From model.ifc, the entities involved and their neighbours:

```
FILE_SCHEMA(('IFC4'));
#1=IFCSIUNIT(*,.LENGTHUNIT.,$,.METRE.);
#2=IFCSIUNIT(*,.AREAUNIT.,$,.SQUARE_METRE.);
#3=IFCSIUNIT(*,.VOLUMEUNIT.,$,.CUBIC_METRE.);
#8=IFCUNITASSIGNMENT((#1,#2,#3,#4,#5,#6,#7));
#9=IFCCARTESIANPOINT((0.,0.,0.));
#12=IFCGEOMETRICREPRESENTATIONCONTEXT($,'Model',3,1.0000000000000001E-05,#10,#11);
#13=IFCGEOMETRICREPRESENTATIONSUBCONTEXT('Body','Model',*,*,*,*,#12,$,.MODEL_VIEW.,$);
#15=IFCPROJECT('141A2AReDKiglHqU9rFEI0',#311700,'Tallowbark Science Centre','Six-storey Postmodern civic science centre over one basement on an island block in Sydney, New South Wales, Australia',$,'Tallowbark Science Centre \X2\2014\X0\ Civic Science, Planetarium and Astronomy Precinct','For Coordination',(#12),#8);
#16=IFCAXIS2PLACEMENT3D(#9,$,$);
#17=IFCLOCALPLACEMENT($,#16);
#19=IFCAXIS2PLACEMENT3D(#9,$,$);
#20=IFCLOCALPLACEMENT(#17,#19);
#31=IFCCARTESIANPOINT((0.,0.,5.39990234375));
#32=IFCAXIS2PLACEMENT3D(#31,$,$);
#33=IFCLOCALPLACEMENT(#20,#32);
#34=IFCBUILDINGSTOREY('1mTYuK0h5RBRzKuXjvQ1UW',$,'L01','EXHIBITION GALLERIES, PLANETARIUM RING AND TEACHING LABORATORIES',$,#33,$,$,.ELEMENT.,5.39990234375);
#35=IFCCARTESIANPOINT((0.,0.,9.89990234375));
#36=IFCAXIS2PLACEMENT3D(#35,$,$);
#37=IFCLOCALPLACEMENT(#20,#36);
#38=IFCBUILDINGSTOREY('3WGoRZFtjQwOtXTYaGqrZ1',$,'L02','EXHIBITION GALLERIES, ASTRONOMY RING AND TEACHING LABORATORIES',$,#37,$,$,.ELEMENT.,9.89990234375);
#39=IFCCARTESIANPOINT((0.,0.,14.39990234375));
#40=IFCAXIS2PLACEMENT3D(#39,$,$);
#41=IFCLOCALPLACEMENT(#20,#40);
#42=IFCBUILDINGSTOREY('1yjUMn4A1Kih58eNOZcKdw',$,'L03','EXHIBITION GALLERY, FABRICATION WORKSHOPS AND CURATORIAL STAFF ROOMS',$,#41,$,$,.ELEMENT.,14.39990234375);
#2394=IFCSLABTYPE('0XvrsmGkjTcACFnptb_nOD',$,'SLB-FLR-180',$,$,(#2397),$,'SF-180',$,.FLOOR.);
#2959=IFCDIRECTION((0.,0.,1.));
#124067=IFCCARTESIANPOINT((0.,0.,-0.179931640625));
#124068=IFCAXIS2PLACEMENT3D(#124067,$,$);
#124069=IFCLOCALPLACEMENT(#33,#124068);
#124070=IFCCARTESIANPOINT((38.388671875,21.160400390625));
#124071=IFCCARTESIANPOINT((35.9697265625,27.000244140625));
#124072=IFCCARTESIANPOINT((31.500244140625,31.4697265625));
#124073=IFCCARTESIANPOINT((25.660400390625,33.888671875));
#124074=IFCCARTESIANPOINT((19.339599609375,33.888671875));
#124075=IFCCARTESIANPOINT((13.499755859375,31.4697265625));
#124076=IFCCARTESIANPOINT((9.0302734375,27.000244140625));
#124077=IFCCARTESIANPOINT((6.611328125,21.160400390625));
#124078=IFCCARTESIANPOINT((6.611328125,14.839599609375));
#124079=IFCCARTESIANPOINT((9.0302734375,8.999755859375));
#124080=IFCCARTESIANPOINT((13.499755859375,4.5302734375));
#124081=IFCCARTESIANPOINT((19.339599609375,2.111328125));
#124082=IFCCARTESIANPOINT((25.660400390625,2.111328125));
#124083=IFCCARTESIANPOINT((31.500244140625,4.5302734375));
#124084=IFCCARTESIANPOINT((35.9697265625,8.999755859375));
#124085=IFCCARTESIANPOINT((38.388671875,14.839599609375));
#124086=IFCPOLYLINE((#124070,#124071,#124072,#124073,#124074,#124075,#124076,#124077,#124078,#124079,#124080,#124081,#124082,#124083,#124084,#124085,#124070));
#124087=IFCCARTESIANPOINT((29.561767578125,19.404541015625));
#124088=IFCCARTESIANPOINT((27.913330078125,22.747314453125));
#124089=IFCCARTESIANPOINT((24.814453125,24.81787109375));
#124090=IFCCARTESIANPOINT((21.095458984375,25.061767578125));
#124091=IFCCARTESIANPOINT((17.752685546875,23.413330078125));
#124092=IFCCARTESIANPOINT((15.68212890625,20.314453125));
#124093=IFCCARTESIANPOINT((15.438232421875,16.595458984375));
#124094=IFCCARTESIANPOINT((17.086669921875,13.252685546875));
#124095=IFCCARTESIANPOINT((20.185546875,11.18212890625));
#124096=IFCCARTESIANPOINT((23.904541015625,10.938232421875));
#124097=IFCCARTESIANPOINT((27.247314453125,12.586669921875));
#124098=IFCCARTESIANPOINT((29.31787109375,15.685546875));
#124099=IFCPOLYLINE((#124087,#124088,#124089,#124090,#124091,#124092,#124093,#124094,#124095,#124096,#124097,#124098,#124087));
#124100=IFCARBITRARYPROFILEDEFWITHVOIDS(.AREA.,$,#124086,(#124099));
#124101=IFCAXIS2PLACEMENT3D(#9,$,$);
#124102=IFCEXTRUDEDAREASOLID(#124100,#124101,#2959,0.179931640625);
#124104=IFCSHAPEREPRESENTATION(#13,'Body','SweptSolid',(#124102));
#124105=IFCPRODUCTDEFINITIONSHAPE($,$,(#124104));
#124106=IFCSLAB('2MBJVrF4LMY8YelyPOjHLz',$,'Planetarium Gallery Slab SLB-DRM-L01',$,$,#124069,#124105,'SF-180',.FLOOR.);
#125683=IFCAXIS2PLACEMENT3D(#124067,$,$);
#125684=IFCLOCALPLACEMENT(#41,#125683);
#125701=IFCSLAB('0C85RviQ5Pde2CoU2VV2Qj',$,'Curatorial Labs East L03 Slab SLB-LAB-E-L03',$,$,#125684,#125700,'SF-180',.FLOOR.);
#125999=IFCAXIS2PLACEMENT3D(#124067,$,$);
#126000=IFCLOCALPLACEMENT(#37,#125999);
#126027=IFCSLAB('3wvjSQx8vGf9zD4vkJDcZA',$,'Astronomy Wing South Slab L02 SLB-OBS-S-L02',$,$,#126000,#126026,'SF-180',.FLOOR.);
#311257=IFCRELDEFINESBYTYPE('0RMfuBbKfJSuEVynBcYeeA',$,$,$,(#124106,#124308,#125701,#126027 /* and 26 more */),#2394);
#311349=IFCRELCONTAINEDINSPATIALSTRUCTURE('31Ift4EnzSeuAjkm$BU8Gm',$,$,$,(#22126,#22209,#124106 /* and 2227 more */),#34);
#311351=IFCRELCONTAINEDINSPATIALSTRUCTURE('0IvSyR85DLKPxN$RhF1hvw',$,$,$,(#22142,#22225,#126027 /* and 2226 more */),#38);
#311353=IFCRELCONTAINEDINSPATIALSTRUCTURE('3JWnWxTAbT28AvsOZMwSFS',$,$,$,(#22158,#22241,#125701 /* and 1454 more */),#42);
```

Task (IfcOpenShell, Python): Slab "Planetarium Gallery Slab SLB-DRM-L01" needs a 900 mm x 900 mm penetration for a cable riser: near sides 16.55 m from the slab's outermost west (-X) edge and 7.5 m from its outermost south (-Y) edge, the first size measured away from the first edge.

```python
import numpy as np
import ifcopenshell
import ifcopenshell.api.feature
import ifcopenshell.api.geometry
import ifcopenshell.api.root
import ifcopenshell.geom
import ifcopenshell.util.placement
import ifcopenshell.util.representation
import ifcopenshell.util.shape
import ifcopenshell.util.unit

model = ifcopenshell.open("model.ifc")
unit_scale = ifcopenshell.util.unit.calculate_unit_scale(model)
settings = ifcopenshell.geom.settings()


def volume(element):
    """Net volume in cubic metres, openings subtracted."""
    shape = ifcopenshell.geom.create_shape(settings, element)
    return ifcopenshell.util.shape.get_volume(shape.geometry)


slab = model.by_guid("2MBJVrF4LMY8YelyPOjHLz")
before = volume(slab)

# Extent in the slab's own axes, in metres. The edges named are its -X and -Y sides.
slab_shape = ifcopenshell.geom.create_shape(settings, slab)
vertices = ifcopenshell.util.shape.get_vertices(slab_shape.geometry)
x_min, y_min, bottom = vertices.min(axis=0)
top = vertices[:, 2].max()

opening = ifcopenshell.api.root.create_entity(model, ifc_class="IfcOpeningElement", name="Cable riser opening", predefined_type="OPENING")
context = ifcopenshell.util.representation.get_context(model, "Model", "Body", "MODEL_VIEW")
width, depth = 0.9, 0.9
outline = [(0.0, 0.0), (width, 0.0), (width, depth), (0.0, depth), (0.0, 0.0)]
# Overshoot both faces by 50 mm so the cut is clean.
shape = ifcopenshell.api.geometry.add_slab_representation(
    model, context=context, depth=top - bottom + 0.1, polyline=outline
)
ifcopenshell.api.geometry.assign_representation(model, product=opening, representation=shape)

matrix = ifcopenshell.util.placement.get_local_placement(slab.ObjectPlacement)
matrix[:, 3] = matrix @ np.append(np.array([x_min + 16.55, y_min + 7.5, bottom - 0.05]) / unit_scale, 1.0)
ifcopenshell.api.geometry.edit_object_placement(model, product=opening, matrix=matrix, is_si=False)
ifcopenshell.api.feature.add_feature(model, feature=opening, element=slab)

after = volume(slab)

print(f"slab volume {before:.3f} -> {after:.3f} m3")

model.write("model_rev.ifc")
```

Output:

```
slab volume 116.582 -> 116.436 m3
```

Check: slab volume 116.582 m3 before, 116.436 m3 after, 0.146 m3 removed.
